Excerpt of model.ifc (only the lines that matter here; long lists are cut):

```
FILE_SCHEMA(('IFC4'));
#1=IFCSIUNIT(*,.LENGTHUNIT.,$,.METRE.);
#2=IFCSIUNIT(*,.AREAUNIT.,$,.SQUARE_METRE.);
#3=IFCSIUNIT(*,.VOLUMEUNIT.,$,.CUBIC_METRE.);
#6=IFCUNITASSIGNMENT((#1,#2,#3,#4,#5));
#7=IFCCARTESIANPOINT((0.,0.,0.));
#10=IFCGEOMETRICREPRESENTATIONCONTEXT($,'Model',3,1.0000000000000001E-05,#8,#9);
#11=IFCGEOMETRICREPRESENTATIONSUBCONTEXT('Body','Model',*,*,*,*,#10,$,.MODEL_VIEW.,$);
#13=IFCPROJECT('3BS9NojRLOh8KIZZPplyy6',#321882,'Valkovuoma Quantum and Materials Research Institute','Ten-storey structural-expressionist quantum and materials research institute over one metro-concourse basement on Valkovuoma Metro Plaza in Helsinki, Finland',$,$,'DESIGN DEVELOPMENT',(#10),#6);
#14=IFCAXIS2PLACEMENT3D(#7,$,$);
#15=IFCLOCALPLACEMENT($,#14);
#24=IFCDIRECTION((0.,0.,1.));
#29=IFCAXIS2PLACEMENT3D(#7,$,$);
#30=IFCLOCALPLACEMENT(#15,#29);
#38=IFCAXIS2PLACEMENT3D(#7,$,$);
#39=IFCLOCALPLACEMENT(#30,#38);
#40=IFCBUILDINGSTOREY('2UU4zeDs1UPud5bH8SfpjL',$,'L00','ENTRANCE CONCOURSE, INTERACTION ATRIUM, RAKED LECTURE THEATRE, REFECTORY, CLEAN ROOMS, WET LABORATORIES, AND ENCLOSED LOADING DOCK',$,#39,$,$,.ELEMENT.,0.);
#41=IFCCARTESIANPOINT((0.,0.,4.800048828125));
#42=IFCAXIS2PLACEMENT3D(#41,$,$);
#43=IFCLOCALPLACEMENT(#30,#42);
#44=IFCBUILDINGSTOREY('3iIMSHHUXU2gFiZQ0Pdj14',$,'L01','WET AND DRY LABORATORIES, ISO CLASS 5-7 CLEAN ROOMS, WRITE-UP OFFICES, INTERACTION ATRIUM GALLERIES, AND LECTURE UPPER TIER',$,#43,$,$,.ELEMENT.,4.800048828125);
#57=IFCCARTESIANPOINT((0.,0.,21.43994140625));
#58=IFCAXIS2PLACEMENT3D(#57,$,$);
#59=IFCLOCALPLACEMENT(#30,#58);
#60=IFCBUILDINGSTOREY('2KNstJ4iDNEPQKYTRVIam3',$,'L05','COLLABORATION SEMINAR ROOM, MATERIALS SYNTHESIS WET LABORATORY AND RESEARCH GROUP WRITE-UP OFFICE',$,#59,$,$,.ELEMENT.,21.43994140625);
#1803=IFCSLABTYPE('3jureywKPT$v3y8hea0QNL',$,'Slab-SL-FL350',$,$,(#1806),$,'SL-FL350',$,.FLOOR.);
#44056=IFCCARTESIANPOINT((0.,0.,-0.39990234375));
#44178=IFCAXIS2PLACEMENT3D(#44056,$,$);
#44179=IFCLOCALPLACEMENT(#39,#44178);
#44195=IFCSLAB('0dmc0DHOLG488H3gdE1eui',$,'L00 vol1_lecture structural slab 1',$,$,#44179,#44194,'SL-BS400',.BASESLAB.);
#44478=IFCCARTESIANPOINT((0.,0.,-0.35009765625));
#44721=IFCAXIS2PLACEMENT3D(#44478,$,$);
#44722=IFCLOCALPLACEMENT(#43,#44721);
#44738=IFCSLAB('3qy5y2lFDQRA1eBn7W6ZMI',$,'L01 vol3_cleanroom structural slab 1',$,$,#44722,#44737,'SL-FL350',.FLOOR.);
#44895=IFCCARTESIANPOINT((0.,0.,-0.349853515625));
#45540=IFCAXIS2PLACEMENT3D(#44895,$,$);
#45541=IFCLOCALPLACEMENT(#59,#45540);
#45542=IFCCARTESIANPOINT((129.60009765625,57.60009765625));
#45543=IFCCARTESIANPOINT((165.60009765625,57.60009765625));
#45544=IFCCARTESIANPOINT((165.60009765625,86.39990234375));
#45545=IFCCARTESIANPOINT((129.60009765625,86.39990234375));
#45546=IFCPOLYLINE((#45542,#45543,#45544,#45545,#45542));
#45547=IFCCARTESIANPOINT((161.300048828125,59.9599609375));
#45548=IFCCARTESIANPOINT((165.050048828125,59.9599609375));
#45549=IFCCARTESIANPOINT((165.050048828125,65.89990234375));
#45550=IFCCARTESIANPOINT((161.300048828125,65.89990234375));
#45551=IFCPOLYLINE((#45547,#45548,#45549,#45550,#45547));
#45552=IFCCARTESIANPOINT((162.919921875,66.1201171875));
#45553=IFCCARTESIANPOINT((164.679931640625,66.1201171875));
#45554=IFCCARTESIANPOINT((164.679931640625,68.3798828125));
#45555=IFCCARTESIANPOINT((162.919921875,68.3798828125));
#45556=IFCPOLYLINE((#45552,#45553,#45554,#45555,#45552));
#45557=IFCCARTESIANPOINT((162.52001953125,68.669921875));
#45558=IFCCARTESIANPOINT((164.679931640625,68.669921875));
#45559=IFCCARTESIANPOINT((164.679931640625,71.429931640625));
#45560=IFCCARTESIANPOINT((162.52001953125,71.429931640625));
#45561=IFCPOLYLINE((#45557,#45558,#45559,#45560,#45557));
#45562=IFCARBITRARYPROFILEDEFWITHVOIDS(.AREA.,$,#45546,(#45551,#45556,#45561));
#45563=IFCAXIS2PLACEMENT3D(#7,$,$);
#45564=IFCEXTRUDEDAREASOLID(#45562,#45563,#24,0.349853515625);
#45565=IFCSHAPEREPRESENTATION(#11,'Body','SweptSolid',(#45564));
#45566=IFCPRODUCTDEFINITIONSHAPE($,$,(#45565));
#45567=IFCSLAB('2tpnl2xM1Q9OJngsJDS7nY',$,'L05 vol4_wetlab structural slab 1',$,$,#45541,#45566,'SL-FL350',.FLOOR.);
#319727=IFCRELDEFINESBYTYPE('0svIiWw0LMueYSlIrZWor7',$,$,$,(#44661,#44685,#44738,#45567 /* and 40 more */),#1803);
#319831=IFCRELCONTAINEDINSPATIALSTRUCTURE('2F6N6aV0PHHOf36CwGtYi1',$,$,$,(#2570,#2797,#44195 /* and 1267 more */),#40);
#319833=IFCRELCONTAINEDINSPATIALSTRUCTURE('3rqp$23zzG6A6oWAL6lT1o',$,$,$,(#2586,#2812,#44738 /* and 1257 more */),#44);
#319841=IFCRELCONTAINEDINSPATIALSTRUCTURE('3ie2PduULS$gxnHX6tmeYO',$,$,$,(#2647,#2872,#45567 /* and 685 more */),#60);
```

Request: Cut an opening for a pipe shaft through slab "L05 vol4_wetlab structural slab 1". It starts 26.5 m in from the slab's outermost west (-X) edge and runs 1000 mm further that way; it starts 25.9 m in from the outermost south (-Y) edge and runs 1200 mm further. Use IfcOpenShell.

```python
import numpy as np
import ifcopenshell
import ifcopenshell.api.feature
import ifcopenshell.api.geometry
import ifcopenshell.api.root
import ifcopenshell.geom
import ifcopenshell.util.placement
import ifcopenshell.util.representation
import ifcopenshell.util.shape
import ifcopenshell.util.unit

model = ifcopenshell.open("model.ifc")
unit_scale = ifcopenshell.util.unit.calculate_unit_scale(model)
settings = ifcopenshell.geom.settings()


def volume(element):
    """Net volume in cubic metres, openings subtracted."""
    shape = ifcopenshell.geom.create_shape(settings, element)
    return ifcopenshell.util.shape.get_volume(shape.geometry)


slab = model.by_guid("2tpnl2xM1Q9OJngsJDS7nY")
before = volume(slab)

# Extent in the slab's own axes, in metres. The edges named are its -X and -Y sides.
slab_shape = ifcopenshell.geom.create_shape(settings, slab)
vertices = ifcopenshell.util.shape.get_vertices(slab_shape.geometry)
x_min, y_min, bottom = vertices.min(axis=0)
top = vertices[:, 2].max()

opening = ifcopenshell.api.root.create_entity(model, ifc_class="IfcOpeningElement", name="Pipe shaft opening", predefined_type="OPENING")
context = ifcopenshell.util.representation.get_context(model, "Model", "Body", "MODEL_VIEW")
width, depth = 1, 1.2
outline = [(0.0, 0.0), (width, 0.0), (width, depth), (0.0, depth), (0.0, 0.0)]
# Overshoot both faces by 50 mm so the cut is clean.
shape = ifcopenshell.api.geometry.add_slab_representation(
    model, context=context, depth=top - bottom + 0.1, polyline=outline
)
ifcopenshell.api.geometry.assign_representation(model, product=opening, representation=shape)

matrix = ifcopenshell.util.placement.get_local_placement(slab.ObjectPlacement)
matrix[:, 3] = matrix @ np.append(np.array([x_min + 26.5, y_min + 25.9, bottom - 0.05]) / unit_scale, 1.0)
ifcopenshell.api.geometry.edit_object_placement(model, product=opening, matrix=matrix, is_si=False)
ifcopenshell.api.feature.add_feature(model, feature=opening, element=slab)

after = volume(slab)

print(f"slab volume {before:.3f} -> {after:.3f} m3")

model.write("model_v2.ifc")
```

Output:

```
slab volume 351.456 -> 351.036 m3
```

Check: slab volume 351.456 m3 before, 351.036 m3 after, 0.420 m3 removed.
